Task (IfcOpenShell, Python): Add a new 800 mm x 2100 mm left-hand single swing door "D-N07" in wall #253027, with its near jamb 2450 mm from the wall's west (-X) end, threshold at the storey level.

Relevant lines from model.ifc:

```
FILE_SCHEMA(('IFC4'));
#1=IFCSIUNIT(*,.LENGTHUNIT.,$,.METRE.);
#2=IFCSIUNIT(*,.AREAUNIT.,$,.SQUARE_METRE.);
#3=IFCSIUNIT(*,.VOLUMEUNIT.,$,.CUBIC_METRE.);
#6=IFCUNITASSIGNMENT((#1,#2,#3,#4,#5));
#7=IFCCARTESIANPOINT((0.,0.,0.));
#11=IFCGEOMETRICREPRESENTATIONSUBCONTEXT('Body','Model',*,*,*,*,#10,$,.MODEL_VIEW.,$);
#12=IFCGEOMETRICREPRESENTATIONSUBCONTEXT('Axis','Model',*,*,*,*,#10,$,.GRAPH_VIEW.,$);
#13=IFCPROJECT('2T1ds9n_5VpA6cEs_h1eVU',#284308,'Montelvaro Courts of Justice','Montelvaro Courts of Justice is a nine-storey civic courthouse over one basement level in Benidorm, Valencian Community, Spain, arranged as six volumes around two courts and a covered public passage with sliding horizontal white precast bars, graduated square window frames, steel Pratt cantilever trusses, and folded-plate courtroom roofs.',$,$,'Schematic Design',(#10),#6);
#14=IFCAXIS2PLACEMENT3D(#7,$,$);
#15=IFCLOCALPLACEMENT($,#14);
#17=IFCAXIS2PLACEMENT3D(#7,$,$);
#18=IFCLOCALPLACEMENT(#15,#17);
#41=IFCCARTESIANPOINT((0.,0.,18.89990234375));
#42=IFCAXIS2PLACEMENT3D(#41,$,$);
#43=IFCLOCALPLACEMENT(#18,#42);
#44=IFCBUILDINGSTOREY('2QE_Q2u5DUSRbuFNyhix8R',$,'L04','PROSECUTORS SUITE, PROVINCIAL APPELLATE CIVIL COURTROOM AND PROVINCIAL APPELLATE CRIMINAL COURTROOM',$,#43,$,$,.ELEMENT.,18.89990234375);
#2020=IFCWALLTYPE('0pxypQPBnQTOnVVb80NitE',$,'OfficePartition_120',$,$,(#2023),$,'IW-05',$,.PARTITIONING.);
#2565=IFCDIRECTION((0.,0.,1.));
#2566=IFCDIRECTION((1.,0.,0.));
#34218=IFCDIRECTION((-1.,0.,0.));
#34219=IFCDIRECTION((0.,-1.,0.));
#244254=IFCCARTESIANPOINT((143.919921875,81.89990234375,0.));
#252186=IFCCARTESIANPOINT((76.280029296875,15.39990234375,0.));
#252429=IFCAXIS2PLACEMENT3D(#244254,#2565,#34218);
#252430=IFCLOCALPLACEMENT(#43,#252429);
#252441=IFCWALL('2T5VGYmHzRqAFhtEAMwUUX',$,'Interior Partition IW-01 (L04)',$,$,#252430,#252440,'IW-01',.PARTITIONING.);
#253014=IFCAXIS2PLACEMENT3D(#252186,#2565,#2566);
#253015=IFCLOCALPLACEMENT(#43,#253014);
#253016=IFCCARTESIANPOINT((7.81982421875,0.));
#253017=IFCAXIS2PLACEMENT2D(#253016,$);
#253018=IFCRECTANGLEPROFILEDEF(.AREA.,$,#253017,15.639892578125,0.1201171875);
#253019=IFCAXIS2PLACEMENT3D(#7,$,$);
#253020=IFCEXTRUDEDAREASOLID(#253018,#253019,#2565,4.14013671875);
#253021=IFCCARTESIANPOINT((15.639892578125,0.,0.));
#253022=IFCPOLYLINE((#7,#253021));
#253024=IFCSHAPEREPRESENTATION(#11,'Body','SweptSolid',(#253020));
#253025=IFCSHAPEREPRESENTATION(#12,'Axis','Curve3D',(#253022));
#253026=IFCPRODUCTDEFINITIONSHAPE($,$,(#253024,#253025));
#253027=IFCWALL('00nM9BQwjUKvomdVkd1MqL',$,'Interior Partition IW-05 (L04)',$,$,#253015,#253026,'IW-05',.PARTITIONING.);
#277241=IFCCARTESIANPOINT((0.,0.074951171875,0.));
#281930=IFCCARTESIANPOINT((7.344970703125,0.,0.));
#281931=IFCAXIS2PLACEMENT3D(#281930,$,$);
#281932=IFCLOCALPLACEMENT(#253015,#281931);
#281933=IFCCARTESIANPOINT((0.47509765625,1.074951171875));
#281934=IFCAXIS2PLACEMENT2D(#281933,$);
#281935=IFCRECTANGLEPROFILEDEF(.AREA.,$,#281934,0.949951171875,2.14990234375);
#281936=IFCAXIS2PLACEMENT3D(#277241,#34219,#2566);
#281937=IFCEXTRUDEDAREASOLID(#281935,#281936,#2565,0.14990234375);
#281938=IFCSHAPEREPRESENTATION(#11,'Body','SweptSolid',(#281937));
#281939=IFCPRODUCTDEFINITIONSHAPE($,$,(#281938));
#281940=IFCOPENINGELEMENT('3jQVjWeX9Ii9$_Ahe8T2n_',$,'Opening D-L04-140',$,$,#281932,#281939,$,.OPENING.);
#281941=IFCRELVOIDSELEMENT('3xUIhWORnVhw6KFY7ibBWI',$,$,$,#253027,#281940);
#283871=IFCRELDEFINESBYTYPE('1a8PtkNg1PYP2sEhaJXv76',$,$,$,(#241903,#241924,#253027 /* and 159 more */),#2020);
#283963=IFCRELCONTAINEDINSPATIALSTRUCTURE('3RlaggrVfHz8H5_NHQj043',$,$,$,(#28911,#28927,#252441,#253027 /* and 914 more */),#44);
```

```python
import numpy as np
import ifcopenshell
import ifcopenshell.api.feature
import ifcopenshell.api.geometry
import ifcopenshell.api.root
import ifcopenshell.api.spatial
import ifcopenshell.geom
import ifcopenshell.util.element
import ifcopenshell.util.placement
import ifcopenshell.util.representation
import ifcopenshell.util.shape
import ifcopenshell.util.unit

model = ifcopenshell.open("model.ifc")
unit_scale = ifcopenshell.util.unit.calculate_unit_scale(model)
settings = ifcopenshell.geom.settings()


def volume(element):
    """Net volume in cubic metres, openings subtracted."""
    shape = ifcopenshell.geom.create_shape(settings, element)
    return ifcopenshell.util.shape.get_volume(shape.geometry)


wall = model.by_guid("00nM9BQwjUKvomdVkd1MqL")
storey = ifcopenshell.util.element.get_container(wall, ifc_class="IfcBuildingStorey")
context = ifcopenshell.util.representation.get_context(model, "Model", "Body", "MODEL_VIEW")
before = volume(wall)

width, height, from_end, sill = 0.8, 2.1, 2.45, 0.0  # metres

# The wall runs along its own X axis, and the end named is its -X end.
wall_shape = ifcopenshell.geom.create_shape(settings, wall)
x, y, z = ifcopenshell.util.shape.get_vertices(wall_shape.geometry).T
start = x.min() + from_end
face, thickness = float(y.min()), float(y.max() - y.min())
wall_matrix = ifcopenshell.util.placement.get_local_placement(wall.ObjectPlacement)
level = ifcopenshell.util.placement.get_local_placement(storey.ObjectPlacement)[2, 3]


def in_wall(x, y):
    """Placement at x, y metres in the wall's axes, at sill height."""
    matrix = wall_matrix.copy()
    matrix[:, 3] = wall_matrix @ np.array([x / unit_scale, y / unit_scale, 0.0, 1.0])
    matrix[2, 3] = level + sill / unit_scale
    return matrix


# Opening: a box that overshoots both wall faces by 50 mm.
opening = ifcopenshell.api.root.create_entity(model, ifc_class="IfcOpeningElement", predefined_type="OPENING")
box = ifcopenshell.api.geometry.add_wall_representation(
    model, context=context, length=width, height=height, thickness=thickness + 0.1
)
ifcopenshell.api.geometry.assign_representation(model, product=opening, representation=box)
ifcopenshell.api.geometry.edit_object_placement(model, product=opening, matrix=in_wall(start, face - 0.05), is_si=False)
ifcopenshell.api.feature.add_feature(model, feature=opening, element=wall)

door = ifcopenshell.api.root.create_entity(model, ifc_class="IfcDoor", name="D-N07", predefined_type="DOOR")
door.OverallWidth, door.OverallHeight = width / unit_scale, height / unit_scale
door.OperationType = "SINGLE_SWING_LEFT"
body = ifcopenshell.api.geometry.add_door_representation(
    model,
    context=context,
    overall_width=door.OverallWidth,
    overall_height=door.OverallHeight,
    operation_type="SINGLE_SWING_LEFT",
    lining_properties={"LiningDepth": thickness / unit_scale, "ThresholdDepth": thickness / unit_scale},
)
ifcopenshell.api.geometry.assign_representation(model, product=door, representation=body)
ifcopenshell.api.spatial.assign_container(model, products=[door], relating_structure=storey)
ifcopenshell.api.feature.add_filling(model, opening=opening, element=door)

# The lining spans the wall, so the door starts at the wall face.
ifcopenshell.api.geometry.edit_object_placement(model, product=door, matrix=in_wall(start, face), is_si=False)

after = volume(wall)

print(f"wall volume {before:.3f} -> {after:.3f} m3")

model.write("model_v2.ifc")
```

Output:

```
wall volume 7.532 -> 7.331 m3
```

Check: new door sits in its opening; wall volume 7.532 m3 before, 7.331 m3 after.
